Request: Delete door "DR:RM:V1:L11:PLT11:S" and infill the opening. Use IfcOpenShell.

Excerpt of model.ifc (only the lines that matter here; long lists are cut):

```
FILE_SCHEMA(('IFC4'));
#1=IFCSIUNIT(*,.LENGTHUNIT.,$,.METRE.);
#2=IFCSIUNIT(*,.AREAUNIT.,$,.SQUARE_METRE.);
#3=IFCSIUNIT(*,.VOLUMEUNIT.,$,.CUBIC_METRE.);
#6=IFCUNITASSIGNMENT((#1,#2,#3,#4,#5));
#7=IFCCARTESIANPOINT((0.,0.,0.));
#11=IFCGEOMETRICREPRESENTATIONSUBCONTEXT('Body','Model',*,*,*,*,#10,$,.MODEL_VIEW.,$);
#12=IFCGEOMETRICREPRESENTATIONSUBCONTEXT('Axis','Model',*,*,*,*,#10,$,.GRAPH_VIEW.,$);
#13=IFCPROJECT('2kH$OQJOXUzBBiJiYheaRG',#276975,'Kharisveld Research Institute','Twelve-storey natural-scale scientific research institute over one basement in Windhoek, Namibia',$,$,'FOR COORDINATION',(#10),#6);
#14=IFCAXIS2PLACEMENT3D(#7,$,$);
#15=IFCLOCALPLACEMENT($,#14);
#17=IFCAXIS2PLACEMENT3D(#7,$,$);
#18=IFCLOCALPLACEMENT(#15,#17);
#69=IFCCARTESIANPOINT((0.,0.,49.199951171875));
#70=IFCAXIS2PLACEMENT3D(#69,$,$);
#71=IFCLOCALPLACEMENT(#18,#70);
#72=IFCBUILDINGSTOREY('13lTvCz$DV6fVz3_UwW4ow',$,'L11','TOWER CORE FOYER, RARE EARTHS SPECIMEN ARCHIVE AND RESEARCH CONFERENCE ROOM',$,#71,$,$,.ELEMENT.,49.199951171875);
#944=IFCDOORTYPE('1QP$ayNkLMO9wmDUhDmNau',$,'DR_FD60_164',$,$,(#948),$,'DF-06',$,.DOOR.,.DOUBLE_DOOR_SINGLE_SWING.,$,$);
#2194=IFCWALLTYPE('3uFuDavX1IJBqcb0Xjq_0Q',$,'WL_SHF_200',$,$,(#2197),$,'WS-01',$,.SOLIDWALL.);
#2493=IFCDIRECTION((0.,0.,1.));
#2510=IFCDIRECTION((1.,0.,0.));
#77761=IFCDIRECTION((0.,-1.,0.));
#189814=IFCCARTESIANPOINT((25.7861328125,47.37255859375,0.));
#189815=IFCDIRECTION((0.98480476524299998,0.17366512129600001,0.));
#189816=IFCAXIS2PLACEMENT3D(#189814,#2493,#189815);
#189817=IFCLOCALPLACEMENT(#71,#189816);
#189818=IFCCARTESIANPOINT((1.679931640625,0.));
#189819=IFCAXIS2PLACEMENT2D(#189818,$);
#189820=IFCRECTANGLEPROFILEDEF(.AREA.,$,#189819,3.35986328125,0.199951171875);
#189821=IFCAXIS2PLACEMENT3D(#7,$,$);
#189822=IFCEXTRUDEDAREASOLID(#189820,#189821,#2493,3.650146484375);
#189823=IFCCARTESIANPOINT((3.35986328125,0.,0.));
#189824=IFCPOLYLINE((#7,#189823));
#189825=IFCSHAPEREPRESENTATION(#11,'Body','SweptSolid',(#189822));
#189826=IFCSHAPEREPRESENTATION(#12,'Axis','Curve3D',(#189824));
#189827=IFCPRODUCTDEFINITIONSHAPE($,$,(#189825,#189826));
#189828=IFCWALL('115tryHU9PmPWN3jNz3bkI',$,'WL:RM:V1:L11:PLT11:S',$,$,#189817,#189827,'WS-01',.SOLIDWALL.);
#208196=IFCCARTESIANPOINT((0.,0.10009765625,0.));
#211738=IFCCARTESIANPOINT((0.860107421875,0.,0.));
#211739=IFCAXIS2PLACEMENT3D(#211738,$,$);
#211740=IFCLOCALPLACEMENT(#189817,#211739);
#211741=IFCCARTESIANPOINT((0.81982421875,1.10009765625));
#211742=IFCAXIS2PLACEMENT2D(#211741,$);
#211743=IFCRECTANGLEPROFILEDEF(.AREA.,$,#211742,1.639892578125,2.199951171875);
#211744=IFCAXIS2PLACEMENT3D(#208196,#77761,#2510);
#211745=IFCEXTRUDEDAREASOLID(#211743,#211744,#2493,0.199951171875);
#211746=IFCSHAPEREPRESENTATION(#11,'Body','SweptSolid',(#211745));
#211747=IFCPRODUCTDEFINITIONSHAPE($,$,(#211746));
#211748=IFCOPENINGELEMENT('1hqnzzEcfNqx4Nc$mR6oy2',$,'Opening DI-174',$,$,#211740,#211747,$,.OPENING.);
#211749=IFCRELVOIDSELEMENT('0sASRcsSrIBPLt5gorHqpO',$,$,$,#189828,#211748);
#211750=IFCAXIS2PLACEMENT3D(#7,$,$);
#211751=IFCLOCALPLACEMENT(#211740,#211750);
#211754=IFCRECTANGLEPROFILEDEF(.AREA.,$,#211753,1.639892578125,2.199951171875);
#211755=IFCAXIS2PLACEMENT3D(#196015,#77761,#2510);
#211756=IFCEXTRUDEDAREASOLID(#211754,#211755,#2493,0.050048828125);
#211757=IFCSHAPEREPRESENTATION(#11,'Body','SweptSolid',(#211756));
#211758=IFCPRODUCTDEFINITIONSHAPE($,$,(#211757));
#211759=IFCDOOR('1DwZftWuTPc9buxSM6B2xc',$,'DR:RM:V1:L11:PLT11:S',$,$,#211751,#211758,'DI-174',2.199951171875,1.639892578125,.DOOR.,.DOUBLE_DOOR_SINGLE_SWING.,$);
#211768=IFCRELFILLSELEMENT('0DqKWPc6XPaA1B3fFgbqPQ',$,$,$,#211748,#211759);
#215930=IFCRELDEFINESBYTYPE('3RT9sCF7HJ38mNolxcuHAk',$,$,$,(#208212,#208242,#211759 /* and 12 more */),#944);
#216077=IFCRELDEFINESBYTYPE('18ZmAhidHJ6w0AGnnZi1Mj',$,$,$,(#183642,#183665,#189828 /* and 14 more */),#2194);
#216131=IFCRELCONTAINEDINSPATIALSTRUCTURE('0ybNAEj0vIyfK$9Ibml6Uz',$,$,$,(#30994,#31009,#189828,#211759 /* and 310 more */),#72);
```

```python
import ifcopenshell
import ifcopenshell.api.feature
import ifcopenshell.api.root
import ifcopenshell.geom
import ifcopenshell.util.shape

model = ifcopenshell.open("model.ifc")
settings = ifcopenshell.geom.settings()


def volume(element):
    """Net volume in cubic metres, openings subtracted."""
    shape = ifcopenshell.geom.create_shape(settings, element)
    return ifcopenshell.util.shape.get_volume(shape.geometry)


door = model.by_guid("1DwZftWuTPc9buxSM6B2xc")
opening = door.FillsVoids[0].RelatingOpeningElement
wall = opening.VoidsElements[0].RelatingBuildingElement
before = volume(wall)

ifcopenshell.api.root.remove_product(model, product=door)
ifcopenshell.api.feature.remove_feature(model, feature=opening)

after = volume(wall)

print(f"wall volume {before:.3f} -> {after:.3f} m3")

model.write("model_v2.ifc")
```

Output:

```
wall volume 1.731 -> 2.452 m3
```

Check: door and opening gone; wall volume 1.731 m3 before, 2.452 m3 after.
